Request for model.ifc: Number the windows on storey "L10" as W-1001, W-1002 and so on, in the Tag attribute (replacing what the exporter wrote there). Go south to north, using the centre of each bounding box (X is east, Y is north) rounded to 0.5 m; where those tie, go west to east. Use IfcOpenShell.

First a look at what the model holds.

```python
import ifcopenshell
import ifcopenshell.util.element
import ifcopenshell.util.placement

model = ifcopenshell.open("model.ifc")
print(model.schema)
storey = next(s for s in model.by_type("IfcBuildingStorey") if s.Name == "L10")
windows = [e for e in ifcopenshell.util.element.get_decomposition(storey) if e.is_a("IfcWindow")]
for e in sorted(windows, key=lambda e: e.id()):
    origin = ifcopenshell.util.placement.get_local_placement(e.ObjectPlacement)[:3, 3]
    print(e.id(), e.Tag, e.Name, origin.round(2) + 0.0, sep=" | ")
```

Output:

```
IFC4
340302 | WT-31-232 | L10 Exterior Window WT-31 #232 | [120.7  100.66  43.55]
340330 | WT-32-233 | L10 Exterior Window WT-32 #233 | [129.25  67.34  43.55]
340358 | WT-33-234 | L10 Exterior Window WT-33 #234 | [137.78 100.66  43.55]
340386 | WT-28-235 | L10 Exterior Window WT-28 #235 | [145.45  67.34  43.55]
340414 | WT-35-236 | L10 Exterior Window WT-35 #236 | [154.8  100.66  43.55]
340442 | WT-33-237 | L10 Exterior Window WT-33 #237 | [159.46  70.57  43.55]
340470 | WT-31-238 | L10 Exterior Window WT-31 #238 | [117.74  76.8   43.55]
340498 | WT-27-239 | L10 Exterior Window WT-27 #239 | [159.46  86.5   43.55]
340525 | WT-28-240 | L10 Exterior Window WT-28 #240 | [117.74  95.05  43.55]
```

```python
import ifcopenshell
import ifcopenshell.geom
import ifcopenshell.util.element
import ifcopenshell.util.shape

model = ifcopenshell.open("model.ifc")
settings = ifcopenshell.geom.settings()
settings.set("use-world-coords", True)


def centre(element):
    shape = ifcopenshell.geom.create_shape(settings, element)
    return ifcopenshell.util.shape.get_bbox_centroid(shape.geometry)


storey = next(s for s in model.by_type("IfcBuildingStorey") if s.Name == "L10")
windows = [e for e in ifcopenshell.util.element.get_decomposition(storey) if e.is_a("IfcWindow")]

# Insertion points can sit at a corner or the storey origin, so sort by the geometry (in metres).
centres = {e: centre(e) for e in windows}
windows.sort(key=lambda e: (round(centres[e][1] / 0.5), centres[e][0]))

for i, e in enumerate(windows, start=1):
    number = f"W-10{i:02d}"
    e.Tag = number
    print(e.id(), number)

model.write("model_v2.ifc")
```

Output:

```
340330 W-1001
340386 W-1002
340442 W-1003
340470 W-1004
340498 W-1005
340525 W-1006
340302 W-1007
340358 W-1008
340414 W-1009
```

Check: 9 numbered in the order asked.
